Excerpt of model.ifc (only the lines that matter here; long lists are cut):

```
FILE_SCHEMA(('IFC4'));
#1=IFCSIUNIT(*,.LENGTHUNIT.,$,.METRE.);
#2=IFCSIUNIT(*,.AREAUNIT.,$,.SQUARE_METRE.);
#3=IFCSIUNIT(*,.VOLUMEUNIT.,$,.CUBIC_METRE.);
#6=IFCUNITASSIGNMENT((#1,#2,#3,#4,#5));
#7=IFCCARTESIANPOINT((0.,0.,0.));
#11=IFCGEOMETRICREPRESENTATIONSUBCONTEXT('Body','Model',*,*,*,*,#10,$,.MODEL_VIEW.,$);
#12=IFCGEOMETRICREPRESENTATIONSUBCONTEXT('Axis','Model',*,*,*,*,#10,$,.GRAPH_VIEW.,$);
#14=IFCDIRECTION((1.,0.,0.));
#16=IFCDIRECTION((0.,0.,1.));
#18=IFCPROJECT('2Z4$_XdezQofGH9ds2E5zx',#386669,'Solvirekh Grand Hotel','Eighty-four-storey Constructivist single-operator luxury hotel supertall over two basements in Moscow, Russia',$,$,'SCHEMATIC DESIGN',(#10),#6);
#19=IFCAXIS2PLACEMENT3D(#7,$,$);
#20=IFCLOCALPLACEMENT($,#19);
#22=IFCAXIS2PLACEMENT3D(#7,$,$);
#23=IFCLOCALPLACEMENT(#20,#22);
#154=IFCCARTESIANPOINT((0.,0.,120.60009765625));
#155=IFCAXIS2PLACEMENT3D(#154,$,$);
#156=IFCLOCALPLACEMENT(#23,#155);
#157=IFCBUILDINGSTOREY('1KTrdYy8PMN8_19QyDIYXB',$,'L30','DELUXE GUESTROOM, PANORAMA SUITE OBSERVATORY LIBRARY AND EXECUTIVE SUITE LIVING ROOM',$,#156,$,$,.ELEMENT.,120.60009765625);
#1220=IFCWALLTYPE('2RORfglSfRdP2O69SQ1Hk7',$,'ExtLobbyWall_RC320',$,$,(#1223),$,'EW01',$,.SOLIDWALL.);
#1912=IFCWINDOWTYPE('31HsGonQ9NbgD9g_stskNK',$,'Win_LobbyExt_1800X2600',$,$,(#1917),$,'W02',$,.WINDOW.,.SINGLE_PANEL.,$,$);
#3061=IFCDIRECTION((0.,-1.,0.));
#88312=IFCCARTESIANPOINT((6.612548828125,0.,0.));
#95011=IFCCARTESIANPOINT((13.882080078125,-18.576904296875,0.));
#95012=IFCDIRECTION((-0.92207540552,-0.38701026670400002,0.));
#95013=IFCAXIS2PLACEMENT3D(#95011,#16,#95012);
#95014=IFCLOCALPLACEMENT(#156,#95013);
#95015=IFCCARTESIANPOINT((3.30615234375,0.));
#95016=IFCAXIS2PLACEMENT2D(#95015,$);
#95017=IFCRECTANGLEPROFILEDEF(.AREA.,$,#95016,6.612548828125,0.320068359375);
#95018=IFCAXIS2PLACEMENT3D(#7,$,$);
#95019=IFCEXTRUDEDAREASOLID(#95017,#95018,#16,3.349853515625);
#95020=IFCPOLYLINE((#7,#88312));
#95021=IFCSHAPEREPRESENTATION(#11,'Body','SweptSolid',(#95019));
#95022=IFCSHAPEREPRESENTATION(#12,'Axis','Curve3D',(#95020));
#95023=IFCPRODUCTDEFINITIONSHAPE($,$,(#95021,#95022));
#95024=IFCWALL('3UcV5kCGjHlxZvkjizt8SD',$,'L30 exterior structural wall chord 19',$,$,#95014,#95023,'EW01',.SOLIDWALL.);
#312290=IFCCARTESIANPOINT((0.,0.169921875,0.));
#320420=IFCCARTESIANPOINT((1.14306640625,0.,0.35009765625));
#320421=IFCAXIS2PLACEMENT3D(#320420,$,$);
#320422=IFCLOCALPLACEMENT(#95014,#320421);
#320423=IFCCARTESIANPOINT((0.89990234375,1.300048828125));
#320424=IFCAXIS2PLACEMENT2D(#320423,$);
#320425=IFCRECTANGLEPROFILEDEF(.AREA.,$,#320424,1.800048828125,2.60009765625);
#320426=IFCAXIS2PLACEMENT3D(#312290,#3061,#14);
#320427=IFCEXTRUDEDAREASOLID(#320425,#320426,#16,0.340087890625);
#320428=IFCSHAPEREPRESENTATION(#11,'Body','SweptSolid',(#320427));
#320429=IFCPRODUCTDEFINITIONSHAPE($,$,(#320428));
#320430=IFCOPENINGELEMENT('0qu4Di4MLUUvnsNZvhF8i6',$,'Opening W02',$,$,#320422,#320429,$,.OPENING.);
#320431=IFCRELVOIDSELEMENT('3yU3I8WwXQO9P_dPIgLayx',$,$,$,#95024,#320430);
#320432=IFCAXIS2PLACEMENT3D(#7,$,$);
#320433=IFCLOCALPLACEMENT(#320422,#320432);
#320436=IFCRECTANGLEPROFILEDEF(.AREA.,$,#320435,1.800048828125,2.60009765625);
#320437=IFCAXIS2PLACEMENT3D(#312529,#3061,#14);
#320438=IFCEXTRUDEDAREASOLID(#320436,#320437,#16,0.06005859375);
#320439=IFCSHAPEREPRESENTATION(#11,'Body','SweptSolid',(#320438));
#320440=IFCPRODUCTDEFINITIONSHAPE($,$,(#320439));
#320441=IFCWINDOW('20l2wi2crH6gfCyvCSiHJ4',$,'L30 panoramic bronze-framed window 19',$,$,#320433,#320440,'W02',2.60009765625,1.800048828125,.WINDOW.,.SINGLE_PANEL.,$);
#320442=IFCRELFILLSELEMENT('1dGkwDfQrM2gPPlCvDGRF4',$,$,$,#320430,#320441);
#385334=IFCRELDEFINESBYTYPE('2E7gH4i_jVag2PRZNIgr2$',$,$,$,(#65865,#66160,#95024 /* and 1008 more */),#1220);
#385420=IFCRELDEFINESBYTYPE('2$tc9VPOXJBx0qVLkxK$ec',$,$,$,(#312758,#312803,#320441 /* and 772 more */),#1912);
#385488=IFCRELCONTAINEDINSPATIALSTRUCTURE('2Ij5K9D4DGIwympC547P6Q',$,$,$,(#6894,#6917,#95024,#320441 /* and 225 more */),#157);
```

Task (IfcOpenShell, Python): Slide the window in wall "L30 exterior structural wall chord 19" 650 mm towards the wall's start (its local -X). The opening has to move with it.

```python
import ifcopenshell
import ifcopenshell.api.geometry
import ifcopenshell.util.placement

model = ifcopenshell.open("model.ifc")

window = model.by_id(320441)
opening = window.FillsVoids[0].RelatingOpeningElement
wall = opening.VoidsElements[0].RelatingBuildingElement

wall_matrix = ifcopenshell.util.placement.get_local_placement(wall.ObjectPlacement)
shift = wall_matrix[:3, 0] * -0.65
before = ifcopenshell.util.placement.get_local_placement(window.ObjectPlacement)[:3, 3].copy()

# The window is placed relative to its opening, so it follows when the opening moves.
matrix = ifcopenshell.util.placement.get_local_placement(opening.ObjectPlacement)
matrix[:3, 3] += shift
ifcopenshell.api.geometry.edit_object_placement(
    model, product=opening, matrix=matrix, is_si=False, should_transform_children=True
)

after = ifcopenshell.util.placement.get_local_placement(window.ObjectPlacement)[:3, 3]
print("window moved by", (after - before).round(3) + 0.0)

model.write("model_v2.ifc")
```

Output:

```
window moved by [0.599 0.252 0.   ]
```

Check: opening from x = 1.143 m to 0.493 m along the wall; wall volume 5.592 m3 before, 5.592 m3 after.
